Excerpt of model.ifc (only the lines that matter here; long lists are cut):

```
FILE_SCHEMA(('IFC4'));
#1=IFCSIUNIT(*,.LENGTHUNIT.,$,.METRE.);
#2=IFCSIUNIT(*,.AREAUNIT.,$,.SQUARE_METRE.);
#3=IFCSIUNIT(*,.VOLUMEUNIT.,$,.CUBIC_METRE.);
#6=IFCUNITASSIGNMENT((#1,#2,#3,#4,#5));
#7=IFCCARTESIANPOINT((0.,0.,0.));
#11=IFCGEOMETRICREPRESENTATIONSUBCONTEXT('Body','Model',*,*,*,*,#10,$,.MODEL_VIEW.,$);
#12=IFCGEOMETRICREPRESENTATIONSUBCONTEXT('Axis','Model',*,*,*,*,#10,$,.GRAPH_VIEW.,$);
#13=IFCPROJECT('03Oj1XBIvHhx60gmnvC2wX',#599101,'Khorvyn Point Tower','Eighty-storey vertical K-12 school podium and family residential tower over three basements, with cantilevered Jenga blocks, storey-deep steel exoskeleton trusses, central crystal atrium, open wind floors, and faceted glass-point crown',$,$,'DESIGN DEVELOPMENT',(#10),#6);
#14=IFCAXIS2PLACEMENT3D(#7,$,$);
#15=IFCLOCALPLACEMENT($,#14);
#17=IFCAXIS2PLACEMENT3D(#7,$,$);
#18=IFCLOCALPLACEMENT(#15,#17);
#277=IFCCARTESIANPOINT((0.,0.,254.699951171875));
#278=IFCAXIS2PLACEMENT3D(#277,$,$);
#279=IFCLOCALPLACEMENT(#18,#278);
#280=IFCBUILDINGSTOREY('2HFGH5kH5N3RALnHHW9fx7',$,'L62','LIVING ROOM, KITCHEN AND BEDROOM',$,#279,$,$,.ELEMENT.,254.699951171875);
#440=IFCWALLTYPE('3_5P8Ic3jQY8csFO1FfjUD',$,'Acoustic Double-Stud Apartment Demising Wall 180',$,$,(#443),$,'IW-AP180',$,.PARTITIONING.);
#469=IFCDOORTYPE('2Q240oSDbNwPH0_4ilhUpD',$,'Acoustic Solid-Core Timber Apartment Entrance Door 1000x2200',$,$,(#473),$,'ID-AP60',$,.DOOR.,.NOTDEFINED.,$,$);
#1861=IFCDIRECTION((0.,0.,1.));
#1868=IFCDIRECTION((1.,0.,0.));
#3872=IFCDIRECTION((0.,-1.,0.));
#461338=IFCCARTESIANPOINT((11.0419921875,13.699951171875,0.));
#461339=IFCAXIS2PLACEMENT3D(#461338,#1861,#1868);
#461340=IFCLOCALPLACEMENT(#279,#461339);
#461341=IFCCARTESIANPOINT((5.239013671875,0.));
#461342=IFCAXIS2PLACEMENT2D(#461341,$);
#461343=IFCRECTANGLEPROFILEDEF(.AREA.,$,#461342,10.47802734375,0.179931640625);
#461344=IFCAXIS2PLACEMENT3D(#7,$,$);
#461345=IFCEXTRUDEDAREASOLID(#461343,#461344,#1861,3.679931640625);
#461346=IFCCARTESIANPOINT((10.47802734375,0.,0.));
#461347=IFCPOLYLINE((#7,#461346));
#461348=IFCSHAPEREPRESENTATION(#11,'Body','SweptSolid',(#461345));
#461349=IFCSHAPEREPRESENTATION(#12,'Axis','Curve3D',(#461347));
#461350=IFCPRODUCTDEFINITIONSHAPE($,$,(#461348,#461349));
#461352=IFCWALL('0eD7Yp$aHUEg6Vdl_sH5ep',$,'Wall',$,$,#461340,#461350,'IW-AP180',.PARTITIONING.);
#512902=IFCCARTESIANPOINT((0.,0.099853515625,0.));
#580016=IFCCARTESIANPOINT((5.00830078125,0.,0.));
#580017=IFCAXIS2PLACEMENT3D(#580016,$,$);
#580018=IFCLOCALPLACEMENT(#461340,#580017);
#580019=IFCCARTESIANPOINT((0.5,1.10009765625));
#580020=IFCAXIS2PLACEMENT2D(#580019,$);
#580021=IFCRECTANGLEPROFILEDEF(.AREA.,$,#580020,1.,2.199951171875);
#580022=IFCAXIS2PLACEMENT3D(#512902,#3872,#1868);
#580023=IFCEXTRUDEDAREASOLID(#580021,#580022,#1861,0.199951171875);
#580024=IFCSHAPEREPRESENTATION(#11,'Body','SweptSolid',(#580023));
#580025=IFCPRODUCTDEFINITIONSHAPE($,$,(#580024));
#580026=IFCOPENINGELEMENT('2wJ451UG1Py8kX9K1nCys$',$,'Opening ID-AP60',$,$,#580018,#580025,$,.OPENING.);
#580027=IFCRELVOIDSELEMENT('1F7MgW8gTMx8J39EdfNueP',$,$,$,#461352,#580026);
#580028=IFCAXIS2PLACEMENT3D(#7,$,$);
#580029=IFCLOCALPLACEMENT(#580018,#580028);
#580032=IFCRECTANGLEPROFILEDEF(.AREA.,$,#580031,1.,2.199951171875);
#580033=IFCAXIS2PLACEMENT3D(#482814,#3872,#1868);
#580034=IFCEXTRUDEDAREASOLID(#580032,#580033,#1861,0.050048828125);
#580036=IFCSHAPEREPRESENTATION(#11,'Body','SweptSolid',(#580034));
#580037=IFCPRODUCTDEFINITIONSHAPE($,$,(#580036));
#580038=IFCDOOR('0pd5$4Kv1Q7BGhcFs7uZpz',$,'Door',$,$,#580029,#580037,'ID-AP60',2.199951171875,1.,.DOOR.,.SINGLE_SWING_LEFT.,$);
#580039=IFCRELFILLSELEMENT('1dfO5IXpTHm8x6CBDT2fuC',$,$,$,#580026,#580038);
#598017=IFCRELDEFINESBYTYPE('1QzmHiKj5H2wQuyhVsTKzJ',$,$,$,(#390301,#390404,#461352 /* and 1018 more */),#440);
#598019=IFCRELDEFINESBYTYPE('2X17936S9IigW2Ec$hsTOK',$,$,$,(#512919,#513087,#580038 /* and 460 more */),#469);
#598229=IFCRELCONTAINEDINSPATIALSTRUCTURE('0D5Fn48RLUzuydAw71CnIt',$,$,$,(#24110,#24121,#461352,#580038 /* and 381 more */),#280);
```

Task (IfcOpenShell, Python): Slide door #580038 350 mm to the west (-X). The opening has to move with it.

```python
import ifcopenshell
import ifcopenshell.api.geometry
import ifcopenshell.util.placement

model = ifcopenshell.open("model.ifc")

door = model.by_guid("0pd5$4Kv1Q7BGhcFs7uZpz")
opening = door.FillsVoids[0].RelatingOpeningElement
wall = opening.VoidsElements[0].RelatingBuildingElement

wall_matrix = ifcopenshell.util.placement.get_local_placement(wall.ObjectPlacement)
shift = wall_matrix[:3, 0] * -0.35
before = ifcopenshell.util.placement.get_local_placement(door.ObjectPlacement)[:3, 3].copy()

# The door is placed relative to its opening, so it follows when the opening moves.
matrix = ifcopenshell.util.placement.get_local_placement(opening.ObjectPlacement)
matrix[:3, 3] += shift
ifcopenshell.api.geometry.edit_object_placement(
    model, product=opening, matrix=matrix, is_si=False, should_transform_children=True
)

after = ifcopenshell.util.placement.get_local_placement(door.ObjectPlacement)[:3, 3]
print("door moved by", (after - before).round(3) + 0.0)

model.write("model-out.ifc")
```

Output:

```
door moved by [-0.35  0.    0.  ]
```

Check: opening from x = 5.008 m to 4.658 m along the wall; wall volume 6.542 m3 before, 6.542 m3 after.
